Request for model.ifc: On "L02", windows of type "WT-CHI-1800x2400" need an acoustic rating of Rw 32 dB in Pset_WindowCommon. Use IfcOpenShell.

First a look at what the model holds.

```python
import ifcopenshell
import ifcopenshell.util.element

model = ifcopenshell.open("model.ifc")
print(model.schema)
storey = next(s for s in model.by_type("IfcBuildingStorey") if s.Name == "L02")
windows = [e for e in ifcopenshell.util.element.get_decomposition(storey) if e.is_a("IfcWindow")]
seen = {}
for e in windows:
    element_type = ifcopenshell.util.element.get_type(e)
    key = (element_type.Name if element_type != e and element_type else None, ifcopenshell.util.element.get_pset(e, "Pset_WindowCommon", "AcousticRating"))
    seen[key] = seen.get(key, 0) + 1
for (name, value), count in sorted(seen.items(), key=str):
    print(count, "x", name, "|", value)
```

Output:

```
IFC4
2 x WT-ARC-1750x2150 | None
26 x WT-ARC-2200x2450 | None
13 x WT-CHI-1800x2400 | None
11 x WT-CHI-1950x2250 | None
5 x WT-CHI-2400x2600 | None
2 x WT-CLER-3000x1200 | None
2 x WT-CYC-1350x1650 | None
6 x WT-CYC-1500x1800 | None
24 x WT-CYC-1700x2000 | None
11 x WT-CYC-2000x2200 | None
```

```python
import ifcopenshell
import ifcopenshell.api.pset
import ifcopenshell.util.element

model = ifcopenshell.open("model.ifc")

storey = next(s for s in model.by_type("IfcBuildingStorey") if s.Name == "L02")
windows = [e for e in ifcopenshell.util.element.get_decomposition(storey) if e.is_a("IfcWindow")]

count = 0
for e in windows:
    element_type = ifcopenshell.util.element.get_type(e)
    if element_type in (None, e) or element_type.Name != "WT-CHI-1800x2400":
        continue
    # add_pset returns the element's existing set when there is one.
    pset = ifcopenshell.api.pset.add_pset(model, product=e, name="Pset_WindowCommon")
    ifcopenshell.api.pset.edit_pset(model, pset=pset, properties={"AcousticRating": "Rw 32 dB"})
    count += 1

print(count, "windows updated")

model.write("model_v2.ifc")
```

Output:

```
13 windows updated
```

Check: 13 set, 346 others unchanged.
